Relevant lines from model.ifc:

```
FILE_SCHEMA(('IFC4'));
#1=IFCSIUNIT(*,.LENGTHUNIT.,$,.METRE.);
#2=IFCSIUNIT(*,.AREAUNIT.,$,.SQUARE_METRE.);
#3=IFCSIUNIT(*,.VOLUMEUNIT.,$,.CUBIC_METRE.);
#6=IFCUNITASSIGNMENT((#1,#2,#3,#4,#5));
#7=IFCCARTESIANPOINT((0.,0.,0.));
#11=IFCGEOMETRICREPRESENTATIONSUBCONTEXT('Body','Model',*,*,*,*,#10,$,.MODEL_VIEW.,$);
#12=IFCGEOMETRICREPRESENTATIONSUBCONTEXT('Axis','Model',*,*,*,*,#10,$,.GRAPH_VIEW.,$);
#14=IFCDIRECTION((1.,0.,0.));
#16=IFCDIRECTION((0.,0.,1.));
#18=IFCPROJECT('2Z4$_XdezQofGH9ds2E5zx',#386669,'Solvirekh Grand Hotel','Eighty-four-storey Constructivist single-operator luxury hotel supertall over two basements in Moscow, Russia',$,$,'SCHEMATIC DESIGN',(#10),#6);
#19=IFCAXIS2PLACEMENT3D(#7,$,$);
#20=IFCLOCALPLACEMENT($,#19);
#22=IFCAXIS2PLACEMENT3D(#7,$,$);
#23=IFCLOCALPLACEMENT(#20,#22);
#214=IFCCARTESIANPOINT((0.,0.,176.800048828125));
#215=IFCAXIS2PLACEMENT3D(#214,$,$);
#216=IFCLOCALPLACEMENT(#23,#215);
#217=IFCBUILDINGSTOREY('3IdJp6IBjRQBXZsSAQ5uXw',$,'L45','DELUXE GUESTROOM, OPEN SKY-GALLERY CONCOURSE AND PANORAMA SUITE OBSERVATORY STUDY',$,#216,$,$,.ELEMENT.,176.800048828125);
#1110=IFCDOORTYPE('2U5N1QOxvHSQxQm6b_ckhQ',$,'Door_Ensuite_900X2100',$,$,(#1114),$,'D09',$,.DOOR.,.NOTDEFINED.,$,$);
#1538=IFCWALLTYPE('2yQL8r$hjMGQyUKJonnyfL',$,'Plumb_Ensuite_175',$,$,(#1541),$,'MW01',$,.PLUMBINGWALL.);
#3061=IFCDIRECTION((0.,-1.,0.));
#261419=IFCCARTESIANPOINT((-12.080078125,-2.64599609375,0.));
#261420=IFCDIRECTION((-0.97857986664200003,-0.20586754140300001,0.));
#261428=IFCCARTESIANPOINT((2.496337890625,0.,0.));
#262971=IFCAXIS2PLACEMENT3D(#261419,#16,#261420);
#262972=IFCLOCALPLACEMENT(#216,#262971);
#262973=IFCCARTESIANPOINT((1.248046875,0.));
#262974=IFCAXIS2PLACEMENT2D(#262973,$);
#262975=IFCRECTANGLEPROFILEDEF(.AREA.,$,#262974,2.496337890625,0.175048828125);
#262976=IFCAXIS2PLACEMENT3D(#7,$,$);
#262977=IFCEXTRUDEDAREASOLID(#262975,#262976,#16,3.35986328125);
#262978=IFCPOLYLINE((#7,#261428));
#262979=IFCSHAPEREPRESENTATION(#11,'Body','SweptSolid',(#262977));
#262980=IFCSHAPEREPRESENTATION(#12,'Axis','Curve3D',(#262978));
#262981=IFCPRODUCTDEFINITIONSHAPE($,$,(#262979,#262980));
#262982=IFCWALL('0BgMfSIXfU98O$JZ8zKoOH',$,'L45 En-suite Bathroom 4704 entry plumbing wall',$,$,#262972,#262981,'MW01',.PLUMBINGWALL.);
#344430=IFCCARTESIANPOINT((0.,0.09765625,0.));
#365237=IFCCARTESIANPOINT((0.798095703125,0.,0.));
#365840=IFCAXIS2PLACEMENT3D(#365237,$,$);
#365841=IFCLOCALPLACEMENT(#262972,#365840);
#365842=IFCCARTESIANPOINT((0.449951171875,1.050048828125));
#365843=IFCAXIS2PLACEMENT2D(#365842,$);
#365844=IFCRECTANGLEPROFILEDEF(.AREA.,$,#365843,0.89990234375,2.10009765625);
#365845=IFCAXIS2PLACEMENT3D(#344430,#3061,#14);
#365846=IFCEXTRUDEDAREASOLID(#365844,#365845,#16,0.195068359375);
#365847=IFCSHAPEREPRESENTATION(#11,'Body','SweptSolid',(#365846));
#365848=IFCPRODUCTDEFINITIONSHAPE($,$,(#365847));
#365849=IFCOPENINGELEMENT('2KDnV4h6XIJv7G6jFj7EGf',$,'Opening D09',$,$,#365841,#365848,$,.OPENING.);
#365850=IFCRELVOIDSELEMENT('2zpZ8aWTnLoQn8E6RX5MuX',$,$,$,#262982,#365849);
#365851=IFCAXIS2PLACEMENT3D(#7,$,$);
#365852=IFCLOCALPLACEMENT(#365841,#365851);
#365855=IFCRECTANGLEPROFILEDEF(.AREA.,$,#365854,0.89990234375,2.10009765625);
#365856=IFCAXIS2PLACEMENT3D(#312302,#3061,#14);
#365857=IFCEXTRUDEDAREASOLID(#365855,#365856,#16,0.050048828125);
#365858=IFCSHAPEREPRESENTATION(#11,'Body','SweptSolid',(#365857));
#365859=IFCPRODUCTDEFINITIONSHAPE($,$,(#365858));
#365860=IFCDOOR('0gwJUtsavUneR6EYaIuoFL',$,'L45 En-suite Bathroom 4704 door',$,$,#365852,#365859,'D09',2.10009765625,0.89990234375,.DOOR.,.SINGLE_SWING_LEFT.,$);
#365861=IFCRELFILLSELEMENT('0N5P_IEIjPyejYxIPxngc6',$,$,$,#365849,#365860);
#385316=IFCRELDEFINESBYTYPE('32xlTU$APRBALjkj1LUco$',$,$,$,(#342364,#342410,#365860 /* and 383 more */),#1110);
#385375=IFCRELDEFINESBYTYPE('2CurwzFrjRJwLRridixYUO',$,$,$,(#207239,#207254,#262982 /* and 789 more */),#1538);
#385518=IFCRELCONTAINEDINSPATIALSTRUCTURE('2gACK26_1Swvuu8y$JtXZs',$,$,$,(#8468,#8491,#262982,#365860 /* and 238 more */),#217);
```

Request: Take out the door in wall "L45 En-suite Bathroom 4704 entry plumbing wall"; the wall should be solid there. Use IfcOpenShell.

```python
import ifcopenshell
import ifcopenshell.api.feature
import ifcopenshell.api.root
import ifcopenshell.geom
import ifcopenshell.util.shape

model = ifcopenshell.open("model.ifc")
settings = ifcopenshell.geom.settings()


def volume(element):
    """Net volume in cubic metres, openings subtracted."""
    shape = ifcopenshell.geom.create_shape(settings, element)
    return ifcopenshell.util.shape.get_volume(shape.geometry)


door = model.by_guid("0gwJUtsavUneR6EYaIuoFL")
opening = door.FillsVoids[0].RelatingOpeningElement
wall = opening.VoidsElements[0].RelatingBuildingElement
before = volume(wall)

ifcopenshell.api.root.remove_product(model, product=door)
ifcopenshell.api.feature.remove_feature(model, feature=opening)

after = volume(wall)

print(f"wall volume {before:.3f} -> {after:.3f} m3")

model.write("model_v2.ifc")
```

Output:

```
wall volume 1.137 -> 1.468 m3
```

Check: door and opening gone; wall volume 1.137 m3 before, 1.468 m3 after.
